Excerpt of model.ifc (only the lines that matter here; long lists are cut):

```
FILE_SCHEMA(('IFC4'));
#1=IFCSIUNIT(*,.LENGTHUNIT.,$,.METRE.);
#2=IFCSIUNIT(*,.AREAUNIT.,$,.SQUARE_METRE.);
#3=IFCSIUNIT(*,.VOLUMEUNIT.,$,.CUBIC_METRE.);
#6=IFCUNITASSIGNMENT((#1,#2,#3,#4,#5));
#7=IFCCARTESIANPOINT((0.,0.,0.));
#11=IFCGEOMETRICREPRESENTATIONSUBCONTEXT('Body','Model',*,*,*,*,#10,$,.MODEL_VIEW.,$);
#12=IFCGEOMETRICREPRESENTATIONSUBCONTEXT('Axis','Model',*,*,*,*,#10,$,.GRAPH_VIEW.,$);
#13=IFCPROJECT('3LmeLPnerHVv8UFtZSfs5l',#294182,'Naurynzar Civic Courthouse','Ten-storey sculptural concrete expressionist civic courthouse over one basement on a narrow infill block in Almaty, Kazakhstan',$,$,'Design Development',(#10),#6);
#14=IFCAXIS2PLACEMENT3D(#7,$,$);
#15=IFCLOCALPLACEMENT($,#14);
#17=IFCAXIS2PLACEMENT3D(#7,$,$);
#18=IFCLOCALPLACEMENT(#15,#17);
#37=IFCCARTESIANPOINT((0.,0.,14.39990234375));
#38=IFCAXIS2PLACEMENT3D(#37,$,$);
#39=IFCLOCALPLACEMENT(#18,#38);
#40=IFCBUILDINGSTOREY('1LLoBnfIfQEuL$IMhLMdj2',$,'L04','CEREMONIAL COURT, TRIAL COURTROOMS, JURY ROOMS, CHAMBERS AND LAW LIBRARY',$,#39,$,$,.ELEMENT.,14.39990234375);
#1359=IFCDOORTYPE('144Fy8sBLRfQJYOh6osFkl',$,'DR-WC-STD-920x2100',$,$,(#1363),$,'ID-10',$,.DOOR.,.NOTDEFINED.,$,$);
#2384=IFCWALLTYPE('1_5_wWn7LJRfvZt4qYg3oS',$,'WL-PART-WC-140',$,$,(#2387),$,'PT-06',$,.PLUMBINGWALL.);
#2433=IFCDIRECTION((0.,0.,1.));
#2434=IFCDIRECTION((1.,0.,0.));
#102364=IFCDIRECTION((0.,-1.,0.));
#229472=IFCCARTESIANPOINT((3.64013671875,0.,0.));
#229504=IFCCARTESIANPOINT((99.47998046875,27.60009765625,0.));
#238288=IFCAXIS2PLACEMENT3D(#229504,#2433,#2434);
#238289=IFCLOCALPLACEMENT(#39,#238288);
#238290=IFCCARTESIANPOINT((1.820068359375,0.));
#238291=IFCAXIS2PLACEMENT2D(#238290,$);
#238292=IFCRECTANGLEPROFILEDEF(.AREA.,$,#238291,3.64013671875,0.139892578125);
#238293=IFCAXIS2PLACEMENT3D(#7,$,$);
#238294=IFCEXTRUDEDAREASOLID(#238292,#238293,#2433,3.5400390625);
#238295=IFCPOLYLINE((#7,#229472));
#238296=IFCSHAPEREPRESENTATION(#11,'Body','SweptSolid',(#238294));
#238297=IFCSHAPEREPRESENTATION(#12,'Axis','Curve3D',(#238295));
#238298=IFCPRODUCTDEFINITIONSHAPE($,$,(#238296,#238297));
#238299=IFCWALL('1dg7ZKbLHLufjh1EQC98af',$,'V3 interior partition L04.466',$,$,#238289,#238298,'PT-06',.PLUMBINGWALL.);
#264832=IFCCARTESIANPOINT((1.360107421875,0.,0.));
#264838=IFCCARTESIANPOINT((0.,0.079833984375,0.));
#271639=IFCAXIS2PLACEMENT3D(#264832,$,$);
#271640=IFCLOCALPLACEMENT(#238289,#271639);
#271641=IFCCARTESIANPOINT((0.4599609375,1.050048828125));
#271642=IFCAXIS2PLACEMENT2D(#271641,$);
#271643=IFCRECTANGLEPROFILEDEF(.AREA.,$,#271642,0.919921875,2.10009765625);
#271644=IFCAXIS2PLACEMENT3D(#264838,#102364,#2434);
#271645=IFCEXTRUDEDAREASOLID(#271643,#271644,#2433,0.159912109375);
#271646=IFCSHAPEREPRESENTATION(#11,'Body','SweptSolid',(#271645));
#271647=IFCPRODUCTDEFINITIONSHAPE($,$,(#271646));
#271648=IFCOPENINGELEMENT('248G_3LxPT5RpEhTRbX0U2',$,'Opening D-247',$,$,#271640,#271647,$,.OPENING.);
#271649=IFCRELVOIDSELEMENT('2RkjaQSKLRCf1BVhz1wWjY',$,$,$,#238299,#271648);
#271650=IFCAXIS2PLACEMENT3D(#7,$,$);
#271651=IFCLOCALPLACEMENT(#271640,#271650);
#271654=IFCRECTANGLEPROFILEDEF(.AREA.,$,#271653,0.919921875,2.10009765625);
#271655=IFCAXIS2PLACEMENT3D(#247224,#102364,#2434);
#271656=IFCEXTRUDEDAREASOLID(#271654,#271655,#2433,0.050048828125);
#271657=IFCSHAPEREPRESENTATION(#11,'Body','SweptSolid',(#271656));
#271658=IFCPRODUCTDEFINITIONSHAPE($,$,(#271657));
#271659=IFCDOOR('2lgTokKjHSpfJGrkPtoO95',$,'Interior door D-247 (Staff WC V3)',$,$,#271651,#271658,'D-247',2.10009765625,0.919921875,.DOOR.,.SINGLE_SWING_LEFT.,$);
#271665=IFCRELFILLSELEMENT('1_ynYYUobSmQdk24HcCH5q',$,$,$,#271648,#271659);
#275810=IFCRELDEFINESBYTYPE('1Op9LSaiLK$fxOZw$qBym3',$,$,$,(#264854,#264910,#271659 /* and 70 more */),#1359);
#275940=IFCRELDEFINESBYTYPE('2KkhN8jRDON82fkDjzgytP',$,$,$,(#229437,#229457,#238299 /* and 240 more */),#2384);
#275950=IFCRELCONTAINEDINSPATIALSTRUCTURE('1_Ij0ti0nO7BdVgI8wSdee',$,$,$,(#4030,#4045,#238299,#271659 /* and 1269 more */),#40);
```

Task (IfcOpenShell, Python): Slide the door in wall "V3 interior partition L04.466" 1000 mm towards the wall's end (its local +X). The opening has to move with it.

```python
import ifcopenshell
import ifcopenshell.api.geometry
import ifcopenshell.util.placement
import ifcopenshell.util.unit

model = ifcopenshell.open("model.ifc")
unit_scale = ifcopenshell.util.unit.calculate_unit_scale(model)

door = model.by_guid("2lgTokKjHSpfJGrkPtoO95")
opening = door.FillsVoids[0].RelatingOpeningElement
wall = opening.VoidsElements[0].RelatingBuildingElement

wall_matrix = ifcopenshell.util.placement.get_local_placement(wall.ObjectPlacement)
shift = wall_matrix[:3, 0] * 1 / unit_scale
before = ifcopenshell.util.placement.get_local_placement(door.ObjectPlacement)[:3, 3].copy()

# The door is placed relative to its opening, so it follows when the opening moves.
matrix = ifcopenshell.util.placement.get_local_placement(opening.ObjectPlacement)
matrix[:3, 3] += shift
ifcopenshell.api.geometry.edit_object_placement(
    model, product=opening, matrix=matrix, is_si=False, should_transform_children=True
)

after = ifcopenshell.util.placement.get_local_placement(door.ObjectPlacement)[:3, 3]
print("door moved by", (after - before).round(3) + 0.0)

model.write("model_rev.ifc")
```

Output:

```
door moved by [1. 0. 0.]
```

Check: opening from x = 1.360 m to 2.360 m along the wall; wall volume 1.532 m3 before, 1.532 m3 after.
